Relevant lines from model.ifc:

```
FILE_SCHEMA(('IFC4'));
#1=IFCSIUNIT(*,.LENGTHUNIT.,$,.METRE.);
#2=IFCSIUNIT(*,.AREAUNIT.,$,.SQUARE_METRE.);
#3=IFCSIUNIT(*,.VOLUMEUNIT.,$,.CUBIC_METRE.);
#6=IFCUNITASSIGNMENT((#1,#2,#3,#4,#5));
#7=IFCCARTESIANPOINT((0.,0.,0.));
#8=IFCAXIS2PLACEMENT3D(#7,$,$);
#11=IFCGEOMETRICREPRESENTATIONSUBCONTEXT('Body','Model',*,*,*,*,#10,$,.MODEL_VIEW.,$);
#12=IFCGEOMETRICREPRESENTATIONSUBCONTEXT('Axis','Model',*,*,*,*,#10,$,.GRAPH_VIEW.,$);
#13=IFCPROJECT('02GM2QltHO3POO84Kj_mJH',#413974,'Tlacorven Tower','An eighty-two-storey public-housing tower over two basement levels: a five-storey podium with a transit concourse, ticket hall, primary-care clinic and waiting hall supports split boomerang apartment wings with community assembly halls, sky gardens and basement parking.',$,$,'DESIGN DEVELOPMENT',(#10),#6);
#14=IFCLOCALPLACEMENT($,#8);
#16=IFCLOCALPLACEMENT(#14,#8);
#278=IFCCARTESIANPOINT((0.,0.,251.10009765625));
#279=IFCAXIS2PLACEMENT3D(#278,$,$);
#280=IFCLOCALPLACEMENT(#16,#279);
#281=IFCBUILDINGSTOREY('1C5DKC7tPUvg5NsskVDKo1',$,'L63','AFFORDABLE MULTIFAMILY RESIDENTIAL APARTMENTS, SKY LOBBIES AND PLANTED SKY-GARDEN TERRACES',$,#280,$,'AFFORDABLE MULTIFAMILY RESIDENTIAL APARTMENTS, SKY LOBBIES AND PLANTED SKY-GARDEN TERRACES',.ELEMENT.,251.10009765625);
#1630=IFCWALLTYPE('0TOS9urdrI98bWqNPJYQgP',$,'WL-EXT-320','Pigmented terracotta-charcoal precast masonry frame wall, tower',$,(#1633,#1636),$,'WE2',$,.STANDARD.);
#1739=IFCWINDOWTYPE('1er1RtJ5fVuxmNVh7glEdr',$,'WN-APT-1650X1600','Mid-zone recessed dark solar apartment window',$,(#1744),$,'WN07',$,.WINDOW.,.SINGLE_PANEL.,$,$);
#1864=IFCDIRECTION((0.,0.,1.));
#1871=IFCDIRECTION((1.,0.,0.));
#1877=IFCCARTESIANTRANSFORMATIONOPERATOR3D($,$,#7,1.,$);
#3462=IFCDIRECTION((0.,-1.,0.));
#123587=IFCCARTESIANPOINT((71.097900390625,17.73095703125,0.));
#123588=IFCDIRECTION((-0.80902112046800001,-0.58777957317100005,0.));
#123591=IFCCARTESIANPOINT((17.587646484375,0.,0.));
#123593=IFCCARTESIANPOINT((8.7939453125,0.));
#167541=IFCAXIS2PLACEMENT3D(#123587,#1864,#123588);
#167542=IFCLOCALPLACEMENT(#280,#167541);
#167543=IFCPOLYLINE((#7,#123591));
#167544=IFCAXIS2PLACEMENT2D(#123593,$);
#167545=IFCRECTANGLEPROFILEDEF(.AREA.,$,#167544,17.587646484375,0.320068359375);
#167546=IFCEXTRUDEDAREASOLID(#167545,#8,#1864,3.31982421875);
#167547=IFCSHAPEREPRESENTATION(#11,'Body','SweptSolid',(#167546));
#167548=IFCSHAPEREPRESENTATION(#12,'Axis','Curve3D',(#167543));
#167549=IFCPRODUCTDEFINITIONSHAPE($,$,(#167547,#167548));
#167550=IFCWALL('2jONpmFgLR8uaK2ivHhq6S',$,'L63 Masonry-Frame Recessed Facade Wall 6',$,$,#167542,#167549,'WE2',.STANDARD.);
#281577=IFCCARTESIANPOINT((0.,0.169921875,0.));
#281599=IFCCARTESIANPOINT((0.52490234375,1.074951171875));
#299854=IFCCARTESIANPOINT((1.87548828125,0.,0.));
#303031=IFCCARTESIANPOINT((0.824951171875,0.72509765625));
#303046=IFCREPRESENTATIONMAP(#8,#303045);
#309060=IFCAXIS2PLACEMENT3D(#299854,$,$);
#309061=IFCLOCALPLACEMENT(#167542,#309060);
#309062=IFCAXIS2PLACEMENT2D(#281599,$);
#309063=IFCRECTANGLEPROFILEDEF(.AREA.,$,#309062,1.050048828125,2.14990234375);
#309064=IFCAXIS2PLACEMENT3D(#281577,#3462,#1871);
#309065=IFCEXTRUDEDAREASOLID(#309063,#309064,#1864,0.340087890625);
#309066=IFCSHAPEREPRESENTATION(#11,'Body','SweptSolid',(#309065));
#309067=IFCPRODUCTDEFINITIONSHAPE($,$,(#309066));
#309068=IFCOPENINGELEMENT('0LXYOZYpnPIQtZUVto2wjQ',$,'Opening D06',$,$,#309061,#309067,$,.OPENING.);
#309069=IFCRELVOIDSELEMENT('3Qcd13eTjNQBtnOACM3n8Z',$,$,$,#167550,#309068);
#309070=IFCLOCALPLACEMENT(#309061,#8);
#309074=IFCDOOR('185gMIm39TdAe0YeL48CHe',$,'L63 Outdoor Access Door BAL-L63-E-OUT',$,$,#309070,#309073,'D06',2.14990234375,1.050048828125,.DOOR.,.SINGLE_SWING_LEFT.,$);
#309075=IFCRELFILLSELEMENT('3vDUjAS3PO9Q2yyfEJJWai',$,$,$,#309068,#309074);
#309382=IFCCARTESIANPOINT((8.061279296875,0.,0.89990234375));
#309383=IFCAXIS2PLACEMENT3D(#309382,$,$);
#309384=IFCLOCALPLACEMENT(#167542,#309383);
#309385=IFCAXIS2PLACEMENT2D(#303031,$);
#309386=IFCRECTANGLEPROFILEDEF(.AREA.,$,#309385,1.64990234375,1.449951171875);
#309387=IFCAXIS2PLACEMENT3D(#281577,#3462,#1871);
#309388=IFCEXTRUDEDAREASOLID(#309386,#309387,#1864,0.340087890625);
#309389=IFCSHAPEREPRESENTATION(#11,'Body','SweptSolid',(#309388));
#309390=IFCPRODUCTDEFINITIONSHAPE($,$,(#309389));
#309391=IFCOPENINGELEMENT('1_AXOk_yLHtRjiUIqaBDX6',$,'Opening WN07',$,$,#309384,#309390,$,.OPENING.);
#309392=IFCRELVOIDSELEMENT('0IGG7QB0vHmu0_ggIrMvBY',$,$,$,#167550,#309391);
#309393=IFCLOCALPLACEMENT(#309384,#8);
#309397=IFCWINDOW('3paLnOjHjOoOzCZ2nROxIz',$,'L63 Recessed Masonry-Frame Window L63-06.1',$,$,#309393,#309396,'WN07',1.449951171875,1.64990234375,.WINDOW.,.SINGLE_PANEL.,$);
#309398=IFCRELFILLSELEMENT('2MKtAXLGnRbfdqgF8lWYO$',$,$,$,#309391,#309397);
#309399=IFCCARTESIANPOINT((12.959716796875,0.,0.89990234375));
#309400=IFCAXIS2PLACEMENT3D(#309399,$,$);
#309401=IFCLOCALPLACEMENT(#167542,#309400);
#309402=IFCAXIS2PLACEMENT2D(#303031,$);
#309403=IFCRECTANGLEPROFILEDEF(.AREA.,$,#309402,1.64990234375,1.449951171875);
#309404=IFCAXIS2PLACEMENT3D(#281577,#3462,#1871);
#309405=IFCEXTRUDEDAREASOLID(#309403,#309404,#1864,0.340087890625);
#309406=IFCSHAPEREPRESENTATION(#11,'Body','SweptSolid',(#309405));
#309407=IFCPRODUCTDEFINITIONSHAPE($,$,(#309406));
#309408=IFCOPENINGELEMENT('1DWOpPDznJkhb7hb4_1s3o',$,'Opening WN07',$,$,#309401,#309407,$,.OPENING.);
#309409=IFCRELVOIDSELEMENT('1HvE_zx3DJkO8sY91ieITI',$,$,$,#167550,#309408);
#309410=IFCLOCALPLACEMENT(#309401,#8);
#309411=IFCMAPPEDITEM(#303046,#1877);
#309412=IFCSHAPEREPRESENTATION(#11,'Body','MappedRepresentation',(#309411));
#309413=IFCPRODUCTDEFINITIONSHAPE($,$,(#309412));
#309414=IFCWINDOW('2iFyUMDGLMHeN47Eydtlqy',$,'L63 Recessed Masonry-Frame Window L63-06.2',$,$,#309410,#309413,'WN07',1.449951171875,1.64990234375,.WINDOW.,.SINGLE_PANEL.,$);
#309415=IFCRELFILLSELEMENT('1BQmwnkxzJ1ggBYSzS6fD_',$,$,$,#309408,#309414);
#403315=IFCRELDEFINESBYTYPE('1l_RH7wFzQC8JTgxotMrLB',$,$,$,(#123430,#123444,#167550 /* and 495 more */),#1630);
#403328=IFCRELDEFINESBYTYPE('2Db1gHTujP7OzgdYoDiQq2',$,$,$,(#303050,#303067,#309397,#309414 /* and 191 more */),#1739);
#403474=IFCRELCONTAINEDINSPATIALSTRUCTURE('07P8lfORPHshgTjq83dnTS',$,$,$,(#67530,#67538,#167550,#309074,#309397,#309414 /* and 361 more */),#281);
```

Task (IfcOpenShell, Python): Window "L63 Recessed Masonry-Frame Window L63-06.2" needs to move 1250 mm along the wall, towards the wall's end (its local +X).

```python
import ifcopenshell
import ifcopenshell.api.geometry
import ifcopenshell.util.placement
import ifcopenshell.util.unit

model = ifcopenshell.open("model.ifc")
unit_scale = ifcopenshell.util.unit.calculate_unit_scale(model)

window = model.by_id(309414)
opening = window.FillsVoids[0].RelatingOpeningElement
wall = opening.VoidsElements[0].RelatingBuildingElement

wall_matrix = ifcopenshell.util.placement.get_local_placement(wall.ObjectPlacement)
shift = wall_matrix[:3, 0] * 1.25 / unit_scale
before = ifcopenshell.util.placement.get_local_placement(window.ObjectPlacement)[:3, 3].copy()

# The window is placed relative to its opening, so it follows when the opening moves.
matrix = ifcopenshell.util.placement.get_local_placement(opening.ObjectPlacement)
matrix[:3, 3] += shift
ifcopenshell.api.geometry.edit_object_placement(
    model, product=opening, matrix=matrix, is_si=False, should_transform_children=True
)

after = ifcopenshell.util.placement.get_local_placement(window.ObjectPlacement)[:3, 3]
print("window moved by", (after - before).round(3) + 0.0)

model.write("model_edited.ifc")
```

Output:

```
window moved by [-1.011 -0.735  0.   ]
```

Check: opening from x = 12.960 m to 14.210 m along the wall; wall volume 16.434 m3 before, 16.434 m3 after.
